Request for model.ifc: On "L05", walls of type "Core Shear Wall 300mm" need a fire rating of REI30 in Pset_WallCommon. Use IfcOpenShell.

First a look at what the model holds.

```python
import ifcopenshell
import ifcopenshell.util.element

model = ifcopenshell.open("model.ifc")
print(model.schema)
storey = next(s for s in model.by_type("IfcBuildingStorey") if s.Name == "L05")
walls = [e for e in ifcopenshell.util.element.get_decomposition(storey) if e.is_a("IfcWall")]
seen = {}
for e in walls:
    element_type = ifcopenshell.util.element.get_type(e)
    key = (element_type.Name if element_type != e and element_type else None, ifcopenshell.util.element.get_pset(e, "Pset_WallCommon", "FireRating"))
    seen[key] = seen.get(key, 0) + 1
for (name, value), count in sorted(seen.items(), key=str):
    print(count, "x", name, "|", value)
```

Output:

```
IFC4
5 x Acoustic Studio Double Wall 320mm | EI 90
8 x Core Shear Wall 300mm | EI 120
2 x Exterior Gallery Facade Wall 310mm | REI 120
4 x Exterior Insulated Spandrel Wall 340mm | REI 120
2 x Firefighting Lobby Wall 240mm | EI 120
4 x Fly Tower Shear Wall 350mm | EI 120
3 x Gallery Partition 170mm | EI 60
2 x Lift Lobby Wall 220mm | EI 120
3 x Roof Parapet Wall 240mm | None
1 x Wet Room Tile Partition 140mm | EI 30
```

```python
import ifcopenshell
import ifcopenshell.api.pset
import ifcopenshell.util.element

model = ifcopenshell.open("model.ifc")

storey = next(s for s in model.by_type("IfcBuildingStorey") if s.Name == "L05")
walls = [e for e in ifcopenshell.util.element.get_decomposition(storey) if e.is_a("IfcWall")]

count = 0
for e in walls:
    element_type = ifcopenshell.util.element.get_type(e)
    if element_type in (None, e) or element_type.Name != "Core Shear Wall 300mm":
        continue
    # add_pset returns the element's existing set when there is one.
    pset = ifcopenshell.api.pset.add_pset(model, product=e, name="Pset_WallCommon")
    ifcopenshell.api.pset.edit_pset(model, pset=pset, properties={"FireRating": "REI30"})
    count += 1

print(count, "walls updated")

model.write("model_updated.ifc")
```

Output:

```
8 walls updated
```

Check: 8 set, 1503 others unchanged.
